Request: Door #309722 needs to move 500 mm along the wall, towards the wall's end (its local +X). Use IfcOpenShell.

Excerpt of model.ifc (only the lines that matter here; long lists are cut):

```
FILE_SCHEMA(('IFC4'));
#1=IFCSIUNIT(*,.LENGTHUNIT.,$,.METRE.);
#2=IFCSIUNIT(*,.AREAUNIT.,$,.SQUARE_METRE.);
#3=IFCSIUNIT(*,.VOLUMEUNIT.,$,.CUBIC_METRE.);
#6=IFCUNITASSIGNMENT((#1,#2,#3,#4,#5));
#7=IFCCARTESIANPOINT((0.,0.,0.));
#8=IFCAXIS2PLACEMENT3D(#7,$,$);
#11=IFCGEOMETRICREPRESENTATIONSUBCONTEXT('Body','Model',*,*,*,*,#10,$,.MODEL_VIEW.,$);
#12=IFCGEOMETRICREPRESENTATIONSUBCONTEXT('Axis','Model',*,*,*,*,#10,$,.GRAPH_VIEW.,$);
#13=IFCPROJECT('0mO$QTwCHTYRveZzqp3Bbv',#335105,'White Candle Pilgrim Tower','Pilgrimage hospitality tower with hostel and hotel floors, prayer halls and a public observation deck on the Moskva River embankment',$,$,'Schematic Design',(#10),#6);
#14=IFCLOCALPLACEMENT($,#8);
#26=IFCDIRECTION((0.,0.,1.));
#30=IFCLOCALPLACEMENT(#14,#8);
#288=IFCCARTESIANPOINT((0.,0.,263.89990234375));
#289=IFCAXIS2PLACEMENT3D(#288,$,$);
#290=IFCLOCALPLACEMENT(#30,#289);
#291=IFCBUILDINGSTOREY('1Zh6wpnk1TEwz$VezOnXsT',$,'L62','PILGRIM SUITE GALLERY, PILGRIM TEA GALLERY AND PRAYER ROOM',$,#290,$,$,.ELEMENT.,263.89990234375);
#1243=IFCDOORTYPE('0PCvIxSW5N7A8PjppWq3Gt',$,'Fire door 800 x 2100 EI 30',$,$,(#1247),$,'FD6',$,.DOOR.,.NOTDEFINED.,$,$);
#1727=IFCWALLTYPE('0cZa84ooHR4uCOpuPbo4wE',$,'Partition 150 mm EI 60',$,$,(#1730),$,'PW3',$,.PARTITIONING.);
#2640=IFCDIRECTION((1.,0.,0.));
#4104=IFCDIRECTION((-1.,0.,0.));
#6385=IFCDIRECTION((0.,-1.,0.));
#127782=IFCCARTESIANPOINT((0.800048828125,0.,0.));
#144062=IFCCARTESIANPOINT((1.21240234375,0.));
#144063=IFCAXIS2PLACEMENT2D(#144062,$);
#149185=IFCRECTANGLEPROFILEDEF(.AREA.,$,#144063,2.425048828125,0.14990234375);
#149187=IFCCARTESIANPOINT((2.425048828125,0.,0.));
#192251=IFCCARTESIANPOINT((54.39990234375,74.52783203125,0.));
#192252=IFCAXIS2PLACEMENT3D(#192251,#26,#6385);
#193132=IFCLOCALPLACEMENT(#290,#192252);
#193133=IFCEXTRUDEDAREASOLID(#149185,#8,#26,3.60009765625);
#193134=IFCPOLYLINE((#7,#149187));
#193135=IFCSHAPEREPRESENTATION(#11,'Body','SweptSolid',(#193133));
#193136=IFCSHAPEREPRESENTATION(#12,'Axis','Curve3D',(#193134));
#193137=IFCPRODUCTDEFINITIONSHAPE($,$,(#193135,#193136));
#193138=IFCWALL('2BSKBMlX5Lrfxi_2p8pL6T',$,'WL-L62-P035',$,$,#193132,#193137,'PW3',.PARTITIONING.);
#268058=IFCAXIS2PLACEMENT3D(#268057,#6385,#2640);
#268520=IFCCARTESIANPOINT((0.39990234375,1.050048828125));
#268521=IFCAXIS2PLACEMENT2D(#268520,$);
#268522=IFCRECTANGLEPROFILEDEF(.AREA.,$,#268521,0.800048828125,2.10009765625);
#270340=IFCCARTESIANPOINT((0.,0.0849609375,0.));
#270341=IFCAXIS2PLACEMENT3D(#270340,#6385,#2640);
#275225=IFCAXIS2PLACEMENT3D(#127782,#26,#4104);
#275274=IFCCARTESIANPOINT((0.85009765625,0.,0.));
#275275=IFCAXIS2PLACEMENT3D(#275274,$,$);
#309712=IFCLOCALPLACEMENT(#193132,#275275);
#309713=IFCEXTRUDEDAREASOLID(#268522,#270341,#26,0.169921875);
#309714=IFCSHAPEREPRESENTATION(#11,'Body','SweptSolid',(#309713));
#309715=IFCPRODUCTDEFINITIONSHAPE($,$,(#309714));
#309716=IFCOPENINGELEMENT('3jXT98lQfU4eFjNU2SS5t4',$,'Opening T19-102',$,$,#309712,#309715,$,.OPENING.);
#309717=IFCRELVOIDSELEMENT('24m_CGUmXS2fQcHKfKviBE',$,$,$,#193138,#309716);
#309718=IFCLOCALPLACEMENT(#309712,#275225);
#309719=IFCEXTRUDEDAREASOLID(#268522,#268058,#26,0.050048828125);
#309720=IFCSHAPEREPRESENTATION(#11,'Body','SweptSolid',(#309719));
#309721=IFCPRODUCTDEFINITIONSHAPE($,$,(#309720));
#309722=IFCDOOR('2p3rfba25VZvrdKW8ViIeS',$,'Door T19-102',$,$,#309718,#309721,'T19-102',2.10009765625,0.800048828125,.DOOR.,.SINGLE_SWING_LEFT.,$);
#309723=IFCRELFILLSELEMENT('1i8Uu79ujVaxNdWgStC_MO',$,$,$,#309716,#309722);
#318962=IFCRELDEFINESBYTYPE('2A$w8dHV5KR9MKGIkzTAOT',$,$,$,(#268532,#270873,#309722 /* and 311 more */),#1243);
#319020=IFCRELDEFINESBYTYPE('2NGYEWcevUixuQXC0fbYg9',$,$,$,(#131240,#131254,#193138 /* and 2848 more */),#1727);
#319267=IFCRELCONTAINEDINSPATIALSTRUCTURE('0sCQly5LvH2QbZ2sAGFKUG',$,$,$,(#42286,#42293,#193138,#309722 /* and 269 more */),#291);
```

```python
import ifcopenshell
import ifcopenshell.api.geometry
import ifcopenshell.util.placement
import ifcopenshell.util.unit

model = ifcopenshell.open("model.ifc")
unit_scale = ifcopenshell.util.unit.calculate_unit_scale(model)

door = model.by_guid("2p3rfba25VZvrdKW8ViIeS")
opening = door.FillsVoids[0].RelatingOpeningElement
wall = opening.VoidsElements[0].RelatingBuildingElement

wall_matrix = ifcopenshell.util.placement.get_local_placement(wall.ObjectPlacement)
shift = wall_matrix[:3, 0] * 0.5 / unit_scale
before = ifcopenshell.util.placement.get_local_placement(door.ObjectPlacement)[:3, 3].copy()

# The door is placed relative to its opening, so it follows when the opening moves.
matrix = ifcopenshell.util.placement.get_local_placement(opening.ObjectPlacement)
matrix[:3, 3] += shift
ifcopenshell.api.geometry.edit_object_placement(
    model, product=opening, matrix=matrix, is_si=False, should_transform_children=True
)

after = ifcopenshell.util.placement.get_local_placement(door.ObjectPlacement)[:3, 3]
print("door moved by", (after - before).round(3) + 0.0)

model.write("model_edited.ifc")
```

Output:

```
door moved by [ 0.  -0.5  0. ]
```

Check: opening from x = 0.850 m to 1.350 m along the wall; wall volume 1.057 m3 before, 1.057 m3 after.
